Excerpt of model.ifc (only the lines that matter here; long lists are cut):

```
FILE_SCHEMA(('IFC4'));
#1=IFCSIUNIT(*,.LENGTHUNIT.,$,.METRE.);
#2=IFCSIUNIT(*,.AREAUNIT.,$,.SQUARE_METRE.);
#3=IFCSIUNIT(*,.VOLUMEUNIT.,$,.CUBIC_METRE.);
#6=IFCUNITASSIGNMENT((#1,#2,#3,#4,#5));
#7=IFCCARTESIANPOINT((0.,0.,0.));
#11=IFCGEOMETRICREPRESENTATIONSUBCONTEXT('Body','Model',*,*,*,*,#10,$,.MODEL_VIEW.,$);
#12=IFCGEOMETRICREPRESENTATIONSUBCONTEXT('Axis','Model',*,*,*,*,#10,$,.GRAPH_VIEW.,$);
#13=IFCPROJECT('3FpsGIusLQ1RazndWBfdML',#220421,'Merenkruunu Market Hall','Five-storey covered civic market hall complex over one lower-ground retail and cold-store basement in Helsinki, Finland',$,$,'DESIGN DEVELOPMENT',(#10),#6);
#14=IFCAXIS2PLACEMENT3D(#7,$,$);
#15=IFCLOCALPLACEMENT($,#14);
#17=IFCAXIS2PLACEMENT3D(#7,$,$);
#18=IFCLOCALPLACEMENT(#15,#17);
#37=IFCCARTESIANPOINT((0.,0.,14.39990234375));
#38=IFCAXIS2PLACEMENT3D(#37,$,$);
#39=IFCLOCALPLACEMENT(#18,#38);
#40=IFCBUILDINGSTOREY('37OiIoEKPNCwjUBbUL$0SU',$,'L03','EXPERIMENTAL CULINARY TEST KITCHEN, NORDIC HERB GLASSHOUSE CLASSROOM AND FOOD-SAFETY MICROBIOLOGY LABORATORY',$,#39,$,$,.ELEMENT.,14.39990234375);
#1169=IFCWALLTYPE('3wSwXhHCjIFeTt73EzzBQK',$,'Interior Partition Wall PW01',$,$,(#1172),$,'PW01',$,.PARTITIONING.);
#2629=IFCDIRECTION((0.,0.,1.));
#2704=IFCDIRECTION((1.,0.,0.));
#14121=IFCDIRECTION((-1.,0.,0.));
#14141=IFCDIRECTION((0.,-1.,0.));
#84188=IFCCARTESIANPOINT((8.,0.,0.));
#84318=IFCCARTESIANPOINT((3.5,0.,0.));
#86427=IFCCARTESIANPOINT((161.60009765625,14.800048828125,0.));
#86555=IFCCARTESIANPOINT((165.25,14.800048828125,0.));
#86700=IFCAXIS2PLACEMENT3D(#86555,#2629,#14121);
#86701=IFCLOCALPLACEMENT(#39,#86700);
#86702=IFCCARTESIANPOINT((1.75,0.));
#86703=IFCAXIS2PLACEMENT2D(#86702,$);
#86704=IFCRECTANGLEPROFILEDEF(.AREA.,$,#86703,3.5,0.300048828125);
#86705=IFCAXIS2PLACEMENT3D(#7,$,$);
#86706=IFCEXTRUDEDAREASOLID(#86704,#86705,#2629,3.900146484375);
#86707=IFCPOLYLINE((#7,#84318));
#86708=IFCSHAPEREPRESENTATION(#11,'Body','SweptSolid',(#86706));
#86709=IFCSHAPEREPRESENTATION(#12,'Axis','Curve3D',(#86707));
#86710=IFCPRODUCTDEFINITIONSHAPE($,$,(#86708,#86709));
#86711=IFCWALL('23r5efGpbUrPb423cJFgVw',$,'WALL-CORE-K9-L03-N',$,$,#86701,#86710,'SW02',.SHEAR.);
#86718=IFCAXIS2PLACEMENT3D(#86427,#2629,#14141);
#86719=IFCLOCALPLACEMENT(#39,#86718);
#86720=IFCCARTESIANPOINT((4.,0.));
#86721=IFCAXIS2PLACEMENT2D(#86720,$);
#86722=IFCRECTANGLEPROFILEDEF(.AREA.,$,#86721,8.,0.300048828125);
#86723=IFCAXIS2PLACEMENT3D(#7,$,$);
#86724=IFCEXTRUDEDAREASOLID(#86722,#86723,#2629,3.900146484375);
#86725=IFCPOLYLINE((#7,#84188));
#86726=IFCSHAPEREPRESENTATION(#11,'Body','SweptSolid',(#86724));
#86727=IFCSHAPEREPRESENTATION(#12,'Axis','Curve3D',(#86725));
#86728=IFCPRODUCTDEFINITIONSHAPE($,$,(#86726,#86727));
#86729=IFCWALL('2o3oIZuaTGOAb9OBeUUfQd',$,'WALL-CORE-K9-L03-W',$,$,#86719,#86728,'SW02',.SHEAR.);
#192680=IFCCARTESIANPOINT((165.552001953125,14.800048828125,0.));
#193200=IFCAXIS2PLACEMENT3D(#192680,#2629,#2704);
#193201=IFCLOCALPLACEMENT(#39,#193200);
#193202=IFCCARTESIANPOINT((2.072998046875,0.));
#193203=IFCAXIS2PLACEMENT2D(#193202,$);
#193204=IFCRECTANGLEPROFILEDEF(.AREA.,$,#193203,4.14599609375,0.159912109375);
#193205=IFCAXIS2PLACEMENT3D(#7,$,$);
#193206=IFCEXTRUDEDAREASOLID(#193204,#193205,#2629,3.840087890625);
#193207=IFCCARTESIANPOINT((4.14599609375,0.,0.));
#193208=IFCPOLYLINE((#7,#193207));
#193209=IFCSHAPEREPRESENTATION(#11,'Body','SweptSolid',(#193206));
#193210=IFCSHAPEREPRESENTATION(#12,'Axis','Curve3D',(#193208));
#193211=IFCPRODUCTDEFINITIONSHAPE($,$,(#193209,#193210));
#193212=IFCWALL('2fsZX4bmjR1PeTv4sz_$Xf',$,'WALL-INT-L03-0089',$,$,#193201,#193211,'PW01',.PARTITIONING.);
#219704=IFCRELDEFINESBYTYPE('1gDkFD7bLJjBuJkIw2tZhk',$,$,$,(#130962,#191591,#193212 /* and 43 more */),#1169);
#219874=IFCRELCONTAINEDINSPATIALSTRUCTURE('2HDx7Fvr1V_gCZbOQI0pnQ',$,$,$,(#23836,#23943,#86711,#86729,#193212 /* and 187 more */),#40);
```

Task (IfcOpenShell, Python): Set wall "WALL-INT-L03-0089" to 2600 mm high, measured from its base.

```python
import ifcopenshell
import ifcopenshell.geom
import ifcopenshell.util.representation
import ifcopenshell.util.shape
import ifcopenshell.util.unit

model = ifcopenshell.open("model.ifc")
unit_scale = ifcopenshell.util.unit.calculate_unit_scale(model)
settings = ifcopenshell.geom.settings()


def volume(element):
    """Net volume in cubic metres, openings subtracted."""
    shape = ifcopenshell.geom.create_shape(settings, element)
    return ifcopenshell.util.shape.get_volume(shape.geometry)


wall = model.by_guid("2fsZX4bmjR1PeTv4sz_$Xf")
before = volume(wall)

body = ifcopenshell.util.representation.get_representation(wall, "Model", "Body")
solid = body.Items[0]
old_height = solid.Depth
solid.Depth = 2.6 / unit_scale
after = volume(wall)

print(f"height {old_height:g} -> {solid.Depth:g}, volume {before:.3f} -> {after:.3f} m3")

model.write("model_updated.ifc")
```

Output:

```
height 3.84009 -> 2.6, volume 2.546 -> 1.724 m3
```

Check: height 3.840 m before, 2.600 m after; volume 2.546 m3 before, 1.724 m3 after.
